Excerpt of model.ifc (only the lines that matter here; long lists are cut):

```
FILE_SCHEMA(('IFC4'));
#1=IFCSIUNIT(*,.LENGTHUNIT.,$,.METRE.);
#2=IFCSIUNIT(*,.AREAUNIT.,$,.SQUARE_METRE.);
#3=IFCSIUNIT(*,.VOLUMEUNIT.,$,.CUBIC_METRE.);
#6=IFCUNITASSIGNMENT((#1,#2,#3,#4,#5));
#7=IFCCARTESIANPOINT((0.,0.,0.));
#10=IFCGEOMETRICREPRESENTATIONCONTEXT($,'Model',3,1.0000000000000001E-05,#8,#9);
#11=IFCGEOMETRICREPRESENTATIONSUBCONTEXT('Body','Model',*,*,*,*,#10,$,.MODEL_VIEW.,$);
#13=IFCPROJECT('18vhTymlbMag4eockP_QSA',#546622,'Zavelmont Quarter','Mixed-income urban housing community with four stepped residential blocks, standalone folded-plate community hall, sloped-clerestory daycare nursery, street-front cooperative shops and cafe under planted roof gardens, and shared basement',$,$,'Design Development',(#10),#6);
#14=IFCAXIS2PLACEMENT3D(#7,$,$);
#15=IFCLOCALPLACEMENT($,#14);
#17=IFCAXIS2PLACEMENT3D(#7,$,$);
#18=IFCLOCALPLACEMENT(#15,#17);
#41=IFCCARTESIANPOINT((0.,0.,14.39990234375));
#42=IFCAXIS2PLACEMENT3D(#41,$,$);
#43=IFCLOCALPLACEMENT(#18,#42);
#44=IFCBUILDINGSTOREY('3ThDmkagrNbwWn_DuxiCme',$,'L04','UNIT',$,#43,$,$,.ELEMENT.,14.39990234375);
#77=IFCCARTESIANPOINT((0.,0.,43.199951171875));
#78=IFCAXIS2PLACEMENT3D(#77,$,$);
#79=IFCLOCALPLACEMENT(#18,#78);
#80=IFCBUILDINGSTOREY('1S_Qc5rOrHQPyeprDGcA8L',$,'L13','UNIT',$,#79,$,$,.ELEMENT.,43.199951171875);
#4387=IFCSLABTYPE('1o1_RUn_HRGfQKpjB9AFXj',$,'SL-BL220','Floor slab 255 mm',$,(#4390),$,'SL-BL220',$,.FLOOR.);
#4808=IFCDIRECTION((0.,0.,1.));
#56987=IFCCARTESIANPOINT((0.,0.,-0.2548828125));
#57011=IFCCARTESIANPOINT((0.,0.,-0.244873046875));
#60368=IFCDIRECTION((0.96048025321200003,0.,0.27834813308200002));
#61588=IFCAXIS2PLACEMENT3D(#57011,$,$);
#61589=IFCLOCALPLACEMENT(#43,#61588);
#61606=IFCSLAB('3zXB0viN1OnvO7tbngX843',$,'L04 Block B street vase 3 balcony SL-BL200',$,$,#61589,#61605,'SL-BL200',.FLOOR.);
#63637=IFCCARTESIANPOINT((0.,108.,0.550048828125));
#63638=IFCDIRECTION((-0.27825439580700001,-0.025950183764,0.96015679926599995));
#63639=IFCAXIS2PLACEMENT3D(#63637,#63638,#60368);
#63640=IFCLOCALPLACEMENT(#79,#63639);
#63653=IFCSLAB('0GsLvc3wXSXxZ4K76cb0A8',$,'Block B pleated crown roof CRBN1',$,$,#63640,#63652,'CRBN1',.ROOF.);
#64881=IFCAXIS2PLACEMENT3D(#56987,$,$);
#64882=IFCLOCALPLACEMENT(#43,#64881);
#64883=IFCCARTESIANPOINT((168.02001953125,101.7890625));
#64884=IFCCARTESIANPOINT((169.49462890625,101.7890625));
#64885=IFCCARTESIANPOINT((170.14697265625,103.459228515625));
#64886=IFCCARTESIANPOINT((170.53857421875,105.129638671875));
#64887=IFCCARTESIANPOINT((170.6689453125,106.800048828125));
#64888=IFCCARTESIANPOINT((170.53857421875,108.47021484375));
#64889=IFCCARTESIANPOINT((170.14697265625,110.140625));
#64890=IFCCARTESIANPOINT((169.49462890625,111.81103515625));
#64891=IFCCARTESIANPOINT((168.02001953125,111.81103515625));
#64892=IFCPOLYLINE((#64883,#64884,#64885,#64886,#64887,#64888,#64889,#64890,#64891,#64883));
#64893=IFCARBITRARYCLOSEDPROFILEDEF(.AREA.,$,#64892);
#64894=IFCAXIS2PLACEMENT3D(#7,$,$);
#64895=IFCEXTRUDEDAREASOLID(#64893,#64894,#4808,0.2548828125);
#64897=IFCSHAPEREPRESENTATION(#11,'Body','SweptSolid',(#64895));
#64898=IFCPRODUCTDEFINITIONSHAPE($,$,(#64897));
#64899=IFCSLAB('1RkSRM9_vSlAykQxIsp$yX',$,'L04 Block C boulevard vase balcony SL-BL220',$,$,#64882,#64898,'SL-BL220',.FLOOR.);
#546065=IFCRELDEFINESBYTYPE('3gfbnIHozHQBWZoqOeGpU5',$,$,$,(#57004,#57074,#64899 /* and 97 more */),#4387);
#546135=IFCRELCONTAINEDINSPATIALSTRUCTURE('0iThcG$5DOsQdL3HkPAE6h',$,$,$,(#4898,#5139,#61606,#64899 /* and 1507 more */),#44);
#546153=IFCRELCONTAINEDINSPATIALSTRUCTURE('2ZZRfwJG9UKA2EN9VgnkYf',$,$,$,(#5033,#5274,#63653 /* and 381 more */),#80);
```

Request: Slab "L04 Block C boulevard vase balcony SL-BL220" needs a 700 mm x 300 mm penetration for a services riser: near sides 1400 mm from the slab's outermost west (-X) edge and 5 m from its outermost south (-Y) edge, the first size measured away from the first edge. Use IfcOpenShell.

```python
import numpy as np
import ifcopenshell
import ifcopenshell.api.feature
import ifcopenshell.api.geometry
import ifcopenshell.api.root
import ifcopenshell.geom
import ifcopenshell.util.placement
import ifcopenshell.util.representation
import ifcopenshell.util.shape
import ifcopenshell.util.unit

model = ifcopenshell.open("model.ifc")
unit_scale = ifcopenshell.util.unit.calculate_unit_scale(model)
settings = ifcopenshell.geom.settings()


def volume(element):
    """Net volume in cubic metres, openings subtracted."""
    shape = ifcopenshell.geom.create_shape(settings, element)
    return ifcopenshell.util.shape.get_volume(shape.geometry)


slab = model.by_id(64899)
before = volume(slab)

# Extent in the slab's own axes, in metres. The edges named are its -X and -Y sides.
slab_shape = ifcopenshell.geom.create_shape(settings, slab)
vertices = ifcopenshell.util.shape.get_vertices(slab_shape.geometry)
x_min, y_min, bottom = vertices.min(axis=0)
top = vertices[:, 2].max()

opening = ifcopenshell.api.root.create_entity(model, ifc_class="IfcOpeningElement", name="Services riser opening", predefined_type="OPENING")
context = ifcopenshell.util.representation.get_context(model, "Model", "Body", "MODEL_VIEW")
width, depth = 0.7, 0.3
outline = [(0.0, 0.0), (width, 0.0), (width, depth), (0.0, depth), (0.0, 0.0)]
# Overshoot both faces by 50 mm so the cut is clean.
shape = ifcopenshell.api.geometry.add_slab_representation(
    model, context=context, depth=top - bottom + 0.1, polyline=outline
)
ifcopenshell.api.geometry.assign_representation(model, product=opening, representation=shape)

matrix = ifcopenshell.util.placement.get_local_placement(slab.ObjectPlacement)
matrix[:, 3] = matrix @ np.append(np.array([x_min + 1.4, y_min + 5, bottom - 0.05]) / unit_scale, 1.0)
ifcopenshell.api.geometry.edit_object_placement(model, product=opening, matrix=matrix, is_si=False)
ifcopenshell.api.feature.add_feature(model, feature=opening, element=slab)

after = volume(slab)

print(f"slab volume {before:.3f} -> {after:.3f} m3")

model.write("model_v2.ifc")
```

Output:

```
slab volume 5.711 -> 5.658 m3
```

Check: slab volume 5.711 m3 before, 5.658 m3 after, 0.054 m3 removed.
